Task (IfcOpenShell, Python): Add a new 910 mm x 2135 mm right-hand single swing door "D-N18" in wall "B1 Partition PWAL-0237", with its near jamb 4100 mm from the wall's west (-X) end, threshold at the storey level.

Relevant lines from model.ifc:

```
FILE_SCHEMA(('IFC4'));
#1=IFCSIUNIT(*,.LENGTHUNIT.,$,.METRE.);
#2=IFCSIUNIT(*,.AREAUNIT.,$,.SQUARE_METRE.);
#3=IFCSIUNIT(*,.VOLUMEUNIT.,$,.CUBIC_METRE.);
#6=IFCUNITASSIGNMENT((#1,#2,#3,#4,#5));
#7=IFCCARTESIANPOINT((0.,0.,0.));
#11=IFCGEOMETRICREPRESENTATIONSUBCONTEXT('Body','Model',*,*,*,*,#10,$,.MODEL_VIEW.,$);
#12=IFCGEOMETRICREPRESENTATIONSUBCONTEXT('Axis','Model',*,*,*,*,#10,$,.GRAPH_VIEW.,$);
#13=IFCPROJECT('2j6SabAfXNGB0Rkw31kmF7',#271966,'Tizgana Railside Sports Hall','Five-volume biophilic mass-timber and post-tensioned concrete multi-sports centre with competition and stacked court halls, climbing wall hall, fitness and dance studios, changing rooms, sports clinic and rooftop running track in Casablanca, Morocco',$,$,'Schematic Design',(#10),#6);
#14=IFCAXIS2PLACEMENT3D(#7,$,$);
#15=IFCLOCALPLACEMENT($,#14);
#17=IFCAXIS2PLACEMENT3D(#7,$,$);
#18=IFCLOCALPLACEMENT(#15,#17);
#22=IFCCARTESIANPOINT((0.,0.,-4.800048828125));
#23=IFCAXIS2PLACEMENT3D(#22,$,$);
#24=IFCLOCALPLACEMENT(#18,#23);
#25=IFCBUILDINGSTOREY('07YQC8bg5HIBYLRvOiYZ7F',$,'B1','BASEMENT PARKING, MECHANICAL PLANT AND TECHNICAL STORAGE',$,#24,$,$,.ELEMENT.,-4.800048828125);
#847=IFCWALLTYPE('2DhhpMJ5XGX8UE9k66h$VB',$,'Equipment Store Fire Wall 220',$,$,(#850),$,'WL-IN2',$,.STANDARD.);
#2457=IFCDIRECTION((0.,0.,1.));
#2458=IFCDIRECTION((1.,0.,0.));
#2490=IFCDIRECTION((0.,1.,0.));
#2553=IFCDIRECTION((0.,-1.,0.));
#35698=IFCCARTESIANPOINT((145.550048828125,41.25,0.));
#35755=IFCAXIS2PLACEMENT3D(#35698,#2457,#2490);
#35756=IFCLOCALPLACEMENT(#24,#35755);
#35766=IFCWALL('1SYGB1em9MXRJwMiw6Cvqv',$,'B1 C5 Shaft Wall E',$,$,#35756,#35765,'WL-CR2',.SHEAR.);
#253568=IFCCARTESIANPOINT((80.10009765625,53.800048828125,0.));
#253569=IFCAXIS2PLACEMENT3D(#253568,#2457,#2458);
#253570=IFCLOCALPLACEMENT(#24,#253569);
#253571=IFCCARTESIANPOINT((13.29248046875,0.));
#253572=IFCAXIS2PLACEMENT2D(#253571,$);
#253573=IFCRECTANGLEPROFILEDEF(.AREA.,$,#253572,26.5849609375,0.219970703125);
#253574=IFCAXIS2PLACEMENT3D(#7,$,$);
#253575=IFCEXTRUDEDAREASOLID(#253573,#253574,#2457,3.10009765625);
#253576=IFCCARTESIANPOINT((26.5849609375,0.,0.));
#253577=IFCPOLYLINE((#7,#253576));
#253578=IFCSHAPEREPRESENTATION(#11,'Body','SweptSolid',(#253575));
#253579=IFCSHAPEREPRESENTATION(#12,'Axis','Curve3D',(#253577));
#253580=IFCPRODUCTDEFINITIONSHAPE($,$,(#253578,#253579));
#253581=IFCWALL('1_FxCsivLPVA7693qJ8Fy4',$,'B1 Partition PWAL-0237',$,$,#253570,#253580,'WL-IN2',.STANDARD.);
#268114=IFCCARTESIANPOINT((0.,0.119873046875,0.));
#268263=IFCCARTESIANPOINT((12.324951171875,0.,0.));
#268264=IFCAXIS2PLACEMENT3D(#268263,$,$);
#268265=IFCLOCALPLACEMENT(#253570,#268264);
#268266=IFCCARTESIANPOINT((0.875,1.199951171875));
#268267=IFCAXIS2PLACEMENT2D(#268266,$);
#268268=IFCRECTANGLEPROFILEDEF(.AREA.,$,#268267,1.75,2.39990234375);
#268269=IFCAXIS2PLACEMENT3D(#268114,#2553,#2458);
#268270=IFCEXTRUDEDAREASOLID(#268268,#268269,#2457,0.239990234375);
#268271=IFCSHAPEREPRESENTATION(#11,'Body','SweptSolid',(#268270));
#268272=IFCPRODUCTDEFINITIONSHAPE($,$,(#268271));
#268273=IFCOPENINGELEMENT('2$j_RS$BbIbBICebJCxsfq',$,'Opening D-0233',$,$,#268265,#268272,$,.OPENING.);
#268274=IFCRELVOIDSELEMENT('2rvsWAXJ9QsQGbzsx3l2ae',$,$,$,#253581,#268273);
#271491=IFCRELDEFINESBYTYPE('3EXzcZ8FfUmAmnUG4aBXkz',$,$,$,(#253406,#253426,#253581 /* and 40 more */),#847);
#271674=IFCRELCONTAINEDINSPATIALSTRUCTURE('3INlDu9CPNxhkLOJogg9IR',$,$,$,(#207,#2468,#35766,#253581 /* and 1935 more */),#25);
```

```python
import numpy as np
import ifcopenshell
import ifcopenshell.api.feature
import ifcopenshell.api.geometry
import ifcopenshell.api.root
import ifcopenshell.api.spatial
import ifcopenshell.geom
import ifcopenshell.util.element
import ifcopenshell.util.placement
import ifcopenshell.util.representation
import ifcopenshell.util.shape
import ifcopenshell.util.unit

model = ifcopenshell.open("model.ifc")
unit_scale = ifcopenshell.util.unit.calculate_unit_scale(model)
settings = ifcopenshell.geom.settings()


def volume(element):
    """Net volume in cubic metres, openings subtracted."""
    shape = ifcopenshell.geom.create_shape(settings, element)
    return ifcopenshell.util.shape.get_volume(shape.geometry)


wall = model.by_guid("1_FxCsivLPVA7693qJ8Fy4")
storey = ifcopenshell.util.element.get_container(wall, ifc_class="IfcBuildingStorey")
context = ifcopenshell.util.representation.get_context(model, "Model", "Body", "MODEL_VIEW")
before = volume(wall)

width, height, from_end, sill = 0.91, 2.135, 4.1, 0.0  # metres

# The wall runs along its own X axis, and the end named is its -X end.
wall_shape = ifcopenshell.geom.create_shape(settings, wall)
x, y, z = ifcopenshell.util.shape.get_vertices(wall_shape.geometry).T
start = x.min() + from_end
face, thickness = float(y.min()), float(y.max() - y.min())
wall_matrix = ifcopenshell.util.placement.get_local_placement(wall.ObjectPlacement)
level = ifcopenshell.util.placement.get_local_placement(storey.ObjectPlacement)[2, 3]


def in_wall(x, y):
    """Placement at x, y metres in the wall's axes, at sill height."""
    matrix = wall_matrix.copy()
    matrix[:, 3] = wall_matrix @ np.array([x / unit_scale, y / unit_scale, 0.0, 1.0])
    matrix[2, 3] = level + sill / unit_scale
    return matrix


# Opening: a box that overshoots both wall faces by 50 mm.
opening = ifcopenshell.api.root.create_entity(model, ifc_class="IfcOpeningElement", predefined_type="OPENING")
box = ifcopenshell.api.geometry.add_wall_representation(
    model, context=context, length=width, height=height, thickness=thickness + 0.1
)
ifcopenshell.api.geometry.assign_representation(model, product=opening, representation=box)
ifcopenshell.api.geometry.edit_object_placement(model, product=opening, matrix=in_wall(start, face - 0.05), is_si=False)
ifcopenshell.api.feature.add_feature(model, feature=opening, element=wall)

door = ifcopenshell.api.root.create_entity(model, ifc_class="IfcDoor", name="D-N18", predefined_type="DOOR")
door.OverallWidth, door.OverallHeight = width / unit_scale, height / unit_scale
door.OperationType = "SINGLE_SWING_RIGHT"
body = ifcopenshell.api.geometry.add_door_representation(
    model,
    context=context,
    overall_width=door.OverallWidth,
    overall_height=door.OverallHeight,
    operation_type="SINGLE_SWING_RIGHT",
    lining_properties={"LiningDepth": thickness / unit_scale, "ThresholdDepth": thickness / unit_scale},
)
ifcopenshell.api.geometry.assign_representation(model, product=door, representation=body)
ifcopenshell.api.spatial.assign_container(model, products=[door], relating_structure=storey)
ifcopenshell.api.feature.add_filling(model, opening=opening, element=door)

# The lining spans the wall, so the door starts at the wall face.
ifcopenshell.api.geometry.edit_object_placement(model, product=door, matrix=in_wall(start, face), is_si=False)

after = volume(wall)

print(f"wall volume {before:.3f} -> {after:.3f} m3")

model.write("model_updated.ifc")
```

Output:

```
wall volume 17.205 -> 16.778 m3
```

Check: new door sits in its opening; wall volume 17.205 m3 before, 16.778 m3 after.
